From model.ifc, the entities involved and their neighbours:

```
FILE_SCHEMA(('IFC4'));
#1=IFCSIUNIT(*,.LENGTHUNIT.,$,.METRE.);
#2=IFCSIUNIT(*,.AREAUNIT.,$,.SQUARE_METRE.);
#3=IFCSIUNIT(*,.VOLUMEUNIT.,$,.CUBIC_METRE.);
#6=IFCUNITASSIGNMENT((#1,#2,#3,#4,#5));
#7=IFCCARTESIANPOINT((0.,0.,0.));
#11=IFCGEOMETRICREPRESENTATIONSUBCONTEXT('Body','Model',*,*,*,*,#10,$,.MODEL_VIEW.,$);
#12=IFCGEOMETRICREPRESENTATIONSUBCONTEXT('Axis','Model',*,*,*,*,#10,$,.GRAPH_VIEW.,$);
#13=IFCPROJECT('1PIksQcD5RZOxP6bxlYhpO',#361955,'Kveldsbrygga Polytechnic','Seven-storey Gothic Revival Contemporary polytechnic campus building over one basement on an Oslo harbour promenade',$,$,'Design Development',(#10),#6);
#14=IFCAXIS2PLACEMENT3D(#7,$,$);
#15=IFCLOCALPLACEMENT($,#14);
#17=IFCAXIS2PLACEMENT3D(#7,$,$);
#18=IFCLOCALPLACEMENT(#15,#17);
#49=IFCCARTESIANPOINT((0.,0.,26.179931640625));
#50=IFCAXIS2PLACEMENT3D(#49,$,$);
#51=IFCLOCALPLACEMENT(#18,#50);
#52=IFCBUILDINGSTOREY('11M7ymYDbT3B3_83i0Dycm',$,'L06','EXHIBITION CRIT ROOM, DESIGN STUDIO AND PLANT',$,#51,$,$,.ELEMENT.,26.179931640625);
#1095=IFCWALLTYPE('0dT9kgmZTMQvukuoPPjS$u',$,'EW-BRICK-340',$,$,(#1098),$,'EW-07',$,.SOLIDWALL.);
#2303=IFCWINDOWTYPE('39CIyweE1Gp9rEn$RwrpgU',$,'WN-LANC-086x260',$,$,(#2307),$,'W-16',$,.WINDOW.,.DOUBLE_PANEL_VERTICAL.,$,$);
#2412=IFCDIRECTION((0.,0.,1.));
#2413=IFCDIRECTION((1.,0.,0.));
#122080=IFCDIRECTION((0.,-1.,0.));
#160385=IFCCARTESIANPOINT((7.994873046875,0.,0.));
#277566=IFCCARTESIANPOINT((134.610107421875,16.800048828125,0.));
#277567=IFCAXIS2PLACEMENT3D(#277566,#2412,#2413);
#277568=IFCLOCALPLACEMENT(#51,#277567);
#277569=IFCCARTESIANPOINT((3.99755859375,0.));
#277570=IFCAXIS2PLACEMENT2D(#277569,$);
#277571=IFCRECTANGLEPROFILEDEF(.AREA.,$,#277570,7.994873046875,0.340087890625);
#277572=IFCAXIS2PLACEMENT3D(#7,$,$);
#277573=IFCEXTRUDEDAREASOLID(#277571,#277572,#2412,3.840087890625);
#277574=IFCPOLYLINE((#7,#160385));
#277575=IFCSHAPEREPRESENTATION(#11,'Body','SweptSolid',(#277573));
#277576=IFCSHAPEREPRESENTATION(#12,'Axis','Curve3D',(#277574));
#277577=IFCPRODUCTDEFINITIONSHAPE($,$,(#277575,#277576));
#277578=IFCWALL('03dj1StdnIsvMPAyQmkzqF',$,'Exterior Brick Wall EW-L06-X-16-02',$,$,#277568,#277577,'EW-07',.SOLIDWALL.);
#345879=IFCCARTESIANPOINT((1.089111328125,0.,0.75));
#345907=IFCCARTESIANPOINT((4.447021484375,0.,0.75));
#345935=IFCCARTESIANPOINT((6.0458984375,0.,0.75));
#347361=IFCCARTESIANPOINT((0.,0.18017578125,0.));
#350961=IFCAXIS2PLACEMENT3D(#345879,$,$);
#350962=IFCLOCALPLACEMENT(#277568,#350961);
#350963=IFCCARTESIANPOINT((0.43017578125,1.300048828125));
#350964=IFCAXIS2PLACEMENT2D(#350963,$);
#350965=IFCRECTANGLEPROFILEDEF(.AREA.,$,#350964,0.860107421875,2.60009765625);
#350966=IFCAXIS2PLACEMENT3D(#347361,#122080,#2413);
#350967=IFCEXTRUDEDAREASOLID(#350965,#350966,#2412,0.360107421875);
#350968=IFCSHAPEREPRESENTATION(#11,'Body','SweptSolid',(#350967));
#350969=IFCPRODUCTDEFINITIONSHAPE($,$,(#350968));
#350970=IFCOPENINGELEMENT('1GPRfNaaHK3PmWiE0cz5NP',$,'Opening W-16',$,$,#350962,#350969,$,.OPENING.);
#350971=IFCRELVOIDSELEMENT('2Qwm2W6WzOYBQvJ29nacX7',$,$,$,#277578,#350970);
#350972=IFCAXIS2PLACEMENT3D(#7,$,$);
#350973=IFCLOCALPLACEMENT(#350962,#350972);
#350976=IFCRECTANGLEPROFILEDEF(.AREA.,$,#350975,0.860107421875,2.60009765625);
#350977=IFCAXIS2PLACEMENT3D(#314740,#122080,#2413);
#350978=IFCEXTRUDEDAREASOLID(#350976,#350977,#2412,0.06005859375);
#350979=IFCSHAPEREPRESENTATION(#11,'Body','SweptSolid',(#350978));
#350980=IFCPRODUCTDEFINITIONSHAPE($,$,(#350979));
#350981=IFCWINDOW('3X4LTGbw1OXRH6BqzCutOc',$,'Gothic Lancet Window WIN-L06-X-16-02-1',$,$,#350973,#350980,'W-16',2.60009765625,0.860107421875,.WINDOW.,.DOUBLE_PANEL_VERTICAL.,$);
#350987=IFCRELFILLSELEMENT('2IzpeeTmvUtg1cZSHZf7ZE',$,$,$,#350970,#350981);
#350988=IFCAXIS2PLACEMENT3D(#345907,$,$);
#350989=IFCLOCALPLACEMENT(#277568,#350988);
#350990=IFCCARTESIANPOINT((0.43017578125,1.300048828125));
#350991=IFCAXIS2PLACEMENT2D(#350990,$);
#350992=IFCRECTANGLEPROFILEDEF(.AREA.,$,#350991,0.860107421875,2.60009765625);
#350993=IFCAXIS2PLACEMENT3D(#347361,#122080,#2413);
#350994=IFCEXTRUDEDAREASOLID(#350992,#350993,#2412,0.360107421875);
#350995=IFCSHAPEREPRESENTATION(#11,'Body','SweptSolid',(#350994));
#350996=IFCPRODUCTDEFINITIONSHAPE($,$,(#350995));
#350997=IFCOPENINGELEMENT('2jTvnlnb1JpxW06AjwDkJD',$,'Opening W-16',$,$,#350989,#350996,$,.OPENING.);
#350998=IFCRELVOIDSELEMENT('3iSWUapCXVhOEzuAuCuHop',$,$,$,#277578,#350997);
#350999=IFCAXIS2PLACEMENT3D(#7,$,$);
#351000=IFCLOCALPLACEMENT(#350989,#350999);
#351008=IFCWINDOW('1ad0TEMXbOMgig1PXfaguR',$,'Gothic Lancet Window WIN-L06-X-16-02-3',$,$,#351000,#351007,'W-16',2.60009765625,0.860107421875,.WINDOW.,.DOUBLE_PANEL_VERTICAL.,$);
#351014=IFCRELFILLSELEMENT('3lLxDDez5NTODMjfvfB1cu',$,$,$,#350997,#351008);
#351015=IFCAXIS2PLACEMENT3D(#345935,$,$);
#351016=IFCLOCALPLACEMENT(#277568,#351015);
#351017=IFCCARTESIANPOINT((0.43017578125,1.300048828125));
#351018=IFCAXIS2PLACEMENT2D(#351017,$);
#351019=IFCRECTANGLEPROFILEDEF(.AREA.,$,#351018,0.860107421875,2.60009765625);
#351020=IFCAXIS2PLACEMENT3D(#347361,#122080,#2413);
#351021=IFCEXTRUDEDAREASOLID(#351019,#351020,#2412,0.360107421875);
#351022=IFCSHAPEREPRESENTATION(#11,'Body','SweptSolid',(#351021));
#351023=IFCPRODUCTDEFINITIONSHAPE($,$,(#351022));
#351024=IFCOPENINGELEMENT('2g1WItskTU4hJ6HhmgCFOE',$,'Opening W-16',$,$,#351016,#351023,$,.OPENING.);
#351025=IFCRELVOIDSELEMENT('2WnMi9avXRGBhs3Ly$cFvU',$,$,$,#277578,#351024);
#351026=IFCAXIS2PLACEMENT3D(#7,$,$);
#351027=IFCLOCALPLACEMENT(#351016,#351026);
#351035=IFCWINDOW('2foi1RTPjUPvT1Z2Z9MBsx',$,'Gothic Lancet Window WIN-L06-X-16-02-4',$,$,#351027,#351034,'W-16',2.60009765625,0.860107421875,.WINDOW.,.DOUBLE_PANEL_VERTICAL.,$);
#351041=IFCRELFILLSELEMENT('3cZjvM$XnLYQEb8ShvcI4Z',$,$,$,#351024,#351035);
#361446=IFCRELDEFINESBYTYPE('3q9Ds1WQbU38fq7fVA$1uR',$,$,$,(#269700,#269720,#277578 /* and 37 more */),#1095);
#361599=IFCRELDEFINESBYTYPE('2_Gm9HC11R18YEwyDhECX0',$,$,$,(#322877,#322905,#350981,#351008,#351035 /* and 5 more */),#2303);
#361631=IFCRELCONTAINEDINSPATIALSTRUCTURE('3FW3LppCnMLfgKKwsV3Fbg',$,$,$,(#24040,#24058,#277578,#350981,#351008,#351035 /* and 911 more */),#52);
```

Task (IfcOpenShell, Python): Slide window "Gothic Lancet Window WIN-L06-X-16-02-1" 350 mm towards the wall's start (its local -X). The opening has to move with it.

```python
import ifcopenshell
import ifcopenshell.api.geometry
import ifcopenshell.util.placement
import ifcopenshell.util.unit

model = ifcopenshell.open("model.ifc")
unit_scale = ifcopenshell.util.unit.calculate_unit_scale(model)

window = model.by_guid("3X4LTGbw1OXRH6BqzCutOc")
opening = window.FillsVoids[0].RelatingOpeningElement
wall = opening.VoidsElements[0].RelatingBuildingElement

wall_matrix = ifcopenshell.util.placement.get_local_placement(wall.ObjectPlacement)
shift = wall_matrix[:3, 0] * -0.35 / unit_scale
before = ifcopenshell.util.placement.get_local_placement(window.ObjectPlacement)[:3, 3].copy()

# The window is placed relative to its opening, so it follows when the opening moves.
matrix = ifcopenshell.util.placement.get_local_placement(opening.ObjectPlacement)
matrix[:3, 3] += shift
ifcopenshell.api.geometry.edit_object_placement(
    model, product=opening, matrix=matrix, is_si=False, should_transform_children=True
)

after = ifcopenshell.util.placement.get_local_placement(window.ObjectPlacement)[:3, 3]
print("window moved by", (after - before).round(3) + 0.0)

model.write("model_v2.ifc")
```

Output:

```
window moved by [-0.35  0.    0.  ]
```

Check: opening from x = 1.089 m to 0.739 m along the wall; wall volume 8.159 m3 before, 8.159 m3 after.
